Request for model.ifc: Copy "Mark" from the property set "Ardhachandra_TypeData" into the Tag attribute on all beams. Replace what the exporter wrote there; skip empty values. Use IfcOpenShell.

First a look at what the model holds.

```python
import ifcopenshell
import ifcopenshell.util.element

model = ifcopenshell.open("model.ifc")
print(model.schema)
beams = model.by_type("IfcBeam")
print(len(beams), "beams")
for e in beams[:8]:
    source = ifcopenshell.util.element.get_pset(e, "Ardhachandra_TypeData", "Mark")
    target = e.Tag
    print(e.id(), repr(source), repr(target), sep=" | ")
```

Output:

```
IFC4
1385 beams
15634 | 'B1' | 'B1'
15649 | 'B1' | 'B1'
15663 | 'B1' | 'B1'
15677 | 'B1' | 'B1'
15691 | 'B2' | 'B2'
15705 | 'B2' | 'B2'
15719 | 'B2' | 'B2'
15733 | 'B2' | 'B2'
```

```python
import ifcopenshell
import ifcopenshell.util.element

model = ifcopenshell.open("model.ifc")

count = 0
for e in model.by_type("IfcBeam"):
    value = ifcopenshell.util.element.get_pset(e, "Ardhachandra_TypeData", "Mark")
    current = e.Tag
    if not value or not value.strip() or current == value:
        continue
    e.Tag = value
    count += 1

print(count, "beams updated")

model.write("model-out.ifc")
```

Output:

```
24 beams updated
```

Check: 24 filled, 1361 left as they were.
